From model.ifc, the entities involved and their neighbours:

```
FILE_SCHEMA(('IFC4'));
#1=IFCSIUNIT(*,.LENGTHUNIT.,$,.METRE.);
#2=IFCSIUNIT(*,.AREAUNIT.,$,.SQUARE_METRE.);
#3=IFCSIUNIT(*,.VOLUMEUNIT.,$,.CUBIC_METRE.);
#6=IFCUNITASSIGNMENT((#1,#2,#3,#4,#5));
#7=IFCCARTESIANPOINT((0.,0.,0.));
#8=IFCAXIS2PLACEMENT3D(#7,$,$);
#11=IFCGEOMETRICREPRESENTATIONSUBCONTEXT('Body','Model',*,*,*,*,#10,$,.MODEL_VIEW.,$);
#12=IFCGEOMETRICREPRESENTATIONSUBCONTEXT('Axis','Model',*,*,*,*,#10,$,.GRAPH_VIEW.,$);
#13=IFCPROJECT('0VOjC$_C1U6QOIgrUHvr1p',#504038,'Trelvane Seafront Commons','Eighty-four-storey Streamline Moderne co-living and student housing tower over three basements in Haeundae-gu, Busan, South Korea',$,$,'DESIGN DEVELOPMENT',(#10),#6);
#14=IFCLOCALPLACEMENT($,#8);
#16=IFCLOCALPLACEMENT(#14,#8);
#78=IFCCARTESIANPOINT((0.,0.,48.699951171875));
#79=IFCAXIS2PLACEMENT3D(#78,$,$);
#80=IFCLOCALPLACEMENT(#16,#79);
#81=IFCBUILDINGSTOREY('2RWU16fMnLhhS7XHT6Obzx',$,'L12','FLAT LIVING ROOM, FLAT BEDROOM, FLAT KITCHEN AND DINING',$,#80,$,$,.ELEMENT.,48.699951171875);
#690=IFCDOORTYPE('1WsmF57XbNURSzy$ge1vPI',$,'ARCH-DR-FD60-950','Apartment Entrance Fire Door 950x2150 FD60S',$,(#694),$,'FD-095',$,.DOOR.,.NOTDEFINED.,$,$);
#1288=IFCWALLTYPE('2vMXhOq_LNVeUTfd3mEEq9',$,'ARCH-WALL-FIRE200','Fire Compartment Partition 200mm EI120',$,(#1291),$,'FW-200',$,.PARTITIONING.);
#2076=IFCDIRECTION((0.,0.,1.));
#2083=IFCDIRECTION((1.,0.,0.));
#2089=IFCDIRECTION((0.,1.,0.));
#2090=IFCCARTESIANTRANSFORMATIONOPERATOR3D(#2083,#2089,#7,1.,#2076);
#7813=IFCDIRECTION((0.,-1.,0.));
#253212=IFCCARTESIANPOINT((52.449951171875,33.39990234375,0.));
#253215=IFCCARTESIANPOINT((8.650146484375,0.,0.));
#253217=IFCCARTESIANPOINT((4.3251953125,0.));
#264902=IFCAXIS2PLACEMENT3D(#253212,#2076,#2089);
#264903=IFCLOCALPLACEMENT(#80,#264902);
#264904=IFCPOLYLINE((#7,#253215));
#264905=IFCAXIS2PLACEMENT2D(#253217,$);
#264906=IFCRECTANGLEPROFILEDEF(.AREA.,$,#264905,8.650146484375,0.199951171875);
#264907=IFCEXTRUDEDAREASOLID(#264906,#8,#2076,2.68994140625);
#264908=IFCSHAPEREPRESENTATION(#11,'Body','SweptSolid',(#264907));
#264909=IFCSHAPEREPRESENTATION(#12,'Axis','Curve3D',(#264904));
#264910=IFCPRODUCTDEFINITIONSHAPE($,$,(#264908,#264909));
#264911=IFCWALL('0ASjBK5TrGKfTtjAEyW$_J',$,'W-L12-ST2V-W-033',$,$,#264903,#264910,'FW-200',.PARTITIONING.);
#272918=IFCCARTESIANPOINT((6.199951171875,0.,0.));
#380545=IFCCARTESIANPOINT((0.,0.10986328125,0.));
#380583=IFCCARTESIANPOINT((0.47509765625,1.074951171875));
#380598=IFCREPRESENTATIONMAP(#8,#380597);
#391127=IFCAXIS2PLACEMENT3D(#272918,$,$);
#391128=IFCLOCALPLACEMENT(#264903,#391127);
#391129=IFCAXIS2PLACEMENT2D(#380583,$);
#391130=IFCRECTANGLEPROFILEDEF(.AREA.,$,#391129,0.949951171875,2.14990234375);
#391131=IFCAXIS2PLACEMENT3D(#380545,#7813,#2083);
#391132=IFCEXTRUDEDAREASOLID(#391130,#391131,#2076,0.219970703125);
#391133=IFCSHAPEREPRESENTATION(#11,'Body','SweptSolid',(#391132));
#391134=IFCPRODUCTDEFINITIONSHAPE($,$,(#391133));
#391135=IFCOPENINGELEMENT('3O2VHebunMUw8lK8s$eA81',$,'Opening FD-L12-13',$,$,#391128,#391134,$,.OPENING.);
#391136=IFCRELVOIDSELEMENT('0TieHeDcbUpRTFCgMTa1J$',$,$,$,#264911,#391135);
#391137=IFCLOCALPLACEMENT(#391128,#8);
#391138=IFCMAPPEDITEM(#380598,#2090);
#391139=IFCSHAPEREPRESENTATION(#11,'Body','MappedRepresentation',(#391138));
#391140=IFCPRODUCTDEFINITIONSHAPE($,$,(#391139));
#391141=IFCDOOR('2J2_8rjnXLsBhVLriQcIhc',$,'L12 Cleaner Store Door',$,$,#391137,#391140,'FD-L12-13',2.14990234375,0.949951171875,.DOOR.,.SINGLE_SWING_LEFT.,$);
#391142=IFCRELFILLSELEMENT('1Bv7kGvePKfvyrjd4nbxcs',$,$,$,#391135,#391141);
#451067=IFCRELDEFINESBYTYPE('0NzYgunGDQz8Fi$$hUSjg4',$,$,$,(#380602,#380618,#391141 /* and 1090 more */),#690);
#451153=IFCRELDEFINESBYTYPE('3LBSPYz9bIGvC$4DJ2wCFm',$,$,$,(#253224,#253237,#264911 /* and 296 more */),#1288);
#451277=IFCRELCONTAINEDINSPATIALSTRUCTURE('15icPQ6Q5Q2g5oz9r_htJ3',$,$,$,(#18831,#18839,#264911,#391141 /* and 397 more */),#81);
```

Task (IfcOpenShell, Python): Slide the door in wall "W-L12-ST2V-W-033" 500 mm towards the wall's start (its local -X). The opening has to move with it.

```python
import ifcopenshell
import ifcopenshell.api.geometry
import ifcopenshell.util.placement
import ifcopenshell.util.unit

model = ifcopenshell.open("model.ifc")
unit_scale = ifcopenshell.util.unit.calculate_unit_scale(model)

door = model.by_guid("2J2_8rjnXLsBhVLriQcIhc")
opening = door.FillsVoids[0].RelatingOpeningElement
wall = opening.VoidsElements[0].RelatingBuildingElement

wall_matrix = ifcopenshell.util.placement.get_local_placement(wall.ObjectPlacement)
shift = wall_matrix[:3, 0] * -0.5 / unit_scale
before = ifcopenshell.util.placement.get_local_placement(door.ObjectPlacement)[:3, 3].copy()

# The door is placed relative to its opening, so it follows when the opening moves.
matrix = ifcopenshell.util.placement.get_local_placement(opening.ObjectPlacement)
matrix[:3, 3] += shift
ifcopenshell.api.geometry.edit_object_placement(
    model, product=opening, matrix=matrix, is_si=False, should_transform_children=True
)

after = ifcopenshell.util.placement.get_local_placement(door.ObjectPlacement)[:3, 3]
print("door moved by", (after - before).round(3) + 0.0)

model.write("model-out.ifc")
```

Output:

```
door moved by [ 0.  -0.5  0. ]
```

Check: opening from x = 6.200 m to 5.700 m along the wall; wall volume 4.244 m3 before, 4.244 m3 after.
